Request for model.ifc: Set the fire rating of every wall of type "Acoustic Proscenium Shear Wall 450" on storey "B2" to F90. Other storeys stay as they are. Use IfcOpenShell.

First a look at what the model holds.

```python
import ifcopenshell
import ifcopenshell.util.element

model = ifcopenshell.open("model.ifc")
print(model.schema)
storey = next(s for s in model.by_type("IfcBuildingStorey") if s.Name == "B2")
walls = [e for e in ifcopenshell.util.element.get_decomposition(storey) if e.is_a("IfcWall")]
seen = {}
for e in walls:
    element_type = ifcopenshell.util.element.get_type(e)
    key = (element_type.Name if element_type != e and element_type else None, ifcopenshell.util.element.get_pset(e, "Pset_WallCommon", "FireRating"))
    seen[key] = seen.get(key, 0) + 1
for (name, value), count in sorted(seen.items(), key=str):
    print(count, "x", name, "|", value)
```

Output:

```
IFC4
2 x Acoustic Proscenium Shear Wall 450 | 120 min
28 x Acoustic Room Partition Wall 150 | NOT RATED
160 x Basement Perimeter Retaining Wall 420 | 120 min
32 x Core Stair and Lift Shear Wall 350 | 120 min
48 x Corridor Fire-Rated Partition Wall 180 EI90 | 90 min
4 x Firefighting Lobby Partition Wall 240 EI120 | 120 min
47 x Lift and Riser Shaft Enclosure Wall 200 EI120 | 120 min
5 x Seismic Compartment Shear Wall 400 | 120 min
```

```python
import ifcopenshell
import ifcopenshell.api.pset
import ifcopenshell.util.element

model = ifcopenshell.open("model.ifc")

storey = next(s for s in model.by_type("IfcBuildingStorey") if s.Name == "B2")
walls = [e for e in ifcopenshell.util.element.get_decomposition(storey) if e.is_a("IfcWall")]

count = 0
for e in walls:
    element_type = ifcopenshell.util.element.get_type(e)
    if element_type in (None, e) or element_type.Name != "Acoustic Proscenium Shear Wall 450":
        continue
    # add_pset returns the element's existing set when there is one.
    pset = ifcopenshell.api.pset.add_pset(model, product=e, name="Pset_WallCommon")
    ifcopenshell.api.pset.edit_pset(model, pset=pset, properties={"FireRating": "F90"})
    count += 1

print(count, "walls updated")

model.write("model_edited.ifc")
```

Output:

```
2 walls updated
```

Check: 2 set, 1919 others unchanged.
